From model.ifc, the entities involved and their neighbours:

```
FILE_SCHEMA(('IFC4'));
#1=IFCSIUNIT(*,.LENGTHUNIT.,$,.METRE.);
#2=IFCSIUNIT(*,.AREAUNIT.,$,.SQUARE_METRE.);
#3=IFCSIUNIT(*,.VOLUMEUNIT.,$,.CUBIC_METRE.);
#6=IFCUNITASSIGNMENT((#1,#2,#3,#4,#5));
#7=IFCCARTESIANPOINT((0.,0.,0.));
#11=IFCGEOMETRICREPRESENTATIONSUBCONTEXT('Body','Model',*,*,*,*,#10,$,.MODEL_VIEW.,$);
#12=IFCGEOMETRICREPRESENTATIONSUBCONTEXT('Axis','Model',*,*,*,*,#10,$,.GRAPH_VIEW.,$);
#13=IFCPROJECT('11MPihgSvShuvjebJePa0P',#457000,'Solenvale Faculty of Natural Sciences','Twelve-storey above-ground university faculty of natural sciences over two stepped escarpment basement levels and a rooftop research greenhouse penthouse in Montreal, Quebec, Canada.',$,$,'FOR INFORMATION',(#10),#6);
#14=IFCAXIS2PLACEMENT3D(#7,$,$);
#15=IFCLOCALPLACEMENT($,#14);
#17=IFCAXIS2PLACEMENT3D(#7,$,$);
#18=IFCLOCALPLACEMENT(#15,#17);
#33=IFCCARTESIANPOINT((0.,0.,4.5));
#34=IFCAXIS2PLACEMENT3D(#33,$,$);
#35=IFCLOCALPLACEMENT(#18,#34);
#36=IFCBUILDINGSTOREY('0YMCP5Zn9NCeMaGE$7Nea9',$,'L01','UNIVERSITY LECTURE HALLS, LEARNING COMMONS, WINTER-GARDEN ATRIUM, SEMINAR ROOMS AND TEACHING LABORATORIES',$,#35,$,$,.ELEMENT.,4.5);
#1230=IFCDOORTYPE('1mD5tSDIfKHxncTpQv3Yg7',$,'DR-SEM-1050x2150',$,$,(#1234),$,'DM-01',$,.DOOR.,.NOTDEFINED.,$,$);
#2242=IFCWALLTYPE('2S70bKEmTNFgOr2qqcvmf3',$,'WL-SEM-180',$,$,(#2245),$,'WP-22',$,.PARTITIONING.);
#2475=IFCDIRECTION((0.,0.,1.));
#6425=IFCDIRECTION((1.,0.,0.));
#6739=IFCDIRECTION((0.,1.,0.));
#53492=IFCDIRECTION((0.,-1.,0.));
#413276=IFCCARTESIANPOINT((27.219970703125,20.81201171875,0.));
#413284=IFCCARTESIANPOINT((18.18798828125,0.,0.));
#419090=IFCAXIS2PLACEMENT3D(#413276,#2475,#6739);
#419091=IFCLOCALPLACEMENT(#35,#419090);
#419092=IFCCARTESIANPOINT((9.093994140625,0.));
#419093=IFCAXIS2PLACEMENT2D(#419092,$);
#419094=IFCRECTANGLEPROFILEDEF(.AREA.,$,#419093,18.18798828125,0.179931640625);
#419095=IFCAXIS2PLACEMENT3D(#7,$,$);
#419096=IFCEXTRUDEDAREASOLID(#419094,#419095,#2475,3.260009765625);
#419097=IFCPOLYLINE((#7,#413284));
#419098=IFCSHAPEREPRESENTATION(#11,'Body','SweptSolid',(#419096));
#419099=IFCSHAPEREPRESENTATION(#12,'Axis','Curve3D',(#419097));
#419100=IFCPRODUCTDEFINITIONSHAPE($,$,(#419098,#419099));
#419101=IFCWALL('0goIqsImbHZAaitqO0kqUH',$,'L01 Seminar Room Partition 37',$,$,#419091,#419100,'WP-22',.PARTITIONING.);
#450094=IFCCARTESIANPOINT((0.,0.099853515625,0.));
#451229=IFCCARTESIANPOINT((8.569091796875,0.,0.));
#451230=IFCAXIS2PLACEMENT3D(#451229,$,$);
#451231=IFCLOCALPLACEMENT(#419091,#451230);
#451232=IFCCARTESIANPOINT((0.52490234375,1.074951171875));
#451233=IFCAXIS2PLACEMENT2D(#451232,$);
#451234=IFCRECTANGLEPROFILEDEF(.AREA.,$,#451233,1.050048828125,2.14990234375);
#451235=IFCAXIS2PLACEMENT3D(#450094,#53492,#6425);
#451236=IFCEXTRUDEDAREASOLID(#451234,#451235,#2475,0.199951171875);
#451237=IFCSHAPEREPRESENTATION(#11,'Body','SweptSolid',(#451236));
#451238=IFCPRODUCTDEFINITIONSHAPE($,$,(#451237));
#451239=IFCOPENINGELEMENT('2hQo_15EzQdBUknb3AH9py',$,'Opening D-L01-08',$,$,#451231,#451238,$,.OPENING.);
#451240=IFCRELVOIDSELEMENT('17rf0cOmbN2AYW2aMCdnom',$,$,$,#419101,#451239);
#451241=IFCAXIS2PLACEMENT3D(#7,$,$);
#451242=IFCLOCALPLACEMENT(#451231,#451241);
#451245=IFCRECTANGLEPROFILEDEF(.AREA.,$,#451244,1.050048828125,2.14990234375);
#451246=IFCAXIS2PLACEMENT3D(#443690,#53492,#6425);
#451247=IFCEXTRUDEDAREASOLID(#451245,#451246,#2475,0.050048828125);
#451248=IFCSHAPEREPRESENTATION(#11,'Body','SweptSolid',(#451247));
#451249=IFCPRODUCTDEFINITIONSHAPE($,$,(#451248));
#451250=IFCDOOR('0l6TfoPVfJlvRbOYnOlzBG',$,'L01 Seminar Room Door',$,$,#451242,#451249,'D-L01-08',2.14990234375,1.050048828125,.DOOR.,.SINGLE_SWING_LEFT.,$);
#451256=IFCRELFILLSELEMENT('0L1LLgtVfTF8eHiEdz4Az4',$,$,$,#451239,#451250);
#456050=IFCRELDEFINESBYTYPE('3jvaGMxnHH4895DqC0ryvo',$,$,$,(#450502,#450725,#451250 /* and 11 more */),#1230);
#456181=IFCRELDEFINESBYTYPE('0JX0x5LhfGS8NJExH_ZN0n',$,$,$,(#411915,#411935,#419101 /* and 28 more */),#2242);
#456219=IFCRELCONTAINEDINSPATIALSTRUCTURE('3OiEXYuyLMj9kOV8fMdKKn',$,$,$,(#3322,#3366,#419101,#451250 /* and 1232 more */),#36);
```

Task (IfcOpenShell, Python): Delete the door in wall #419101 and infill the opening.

```python
import ifcopenshell
import ifcopenshell.api.feature
import ifcopenshell.api.root
import ifcopenshell.geom
import ifcopenshell.util.shape

model = ifcopenshell.open("model.ifc")
settings = ifcopenshell.geom.settings()


def volume(element):
    """Net volume in cubic metres, openings subtracted."""
    shape = ifcopenshell.geom.create_shape(settings, element)
    return ifcopenshell.util.shape.get_volume(shape.geometry)


door = model.by_guid("0l6TfoPVfJlvRbOYnOlzBG")
opening = door.FillsVoids[0].RelatingOpeningElement
wall = opening.VoidsElements[0].RelatingBuildingElement
before = volume(wall)

ifcopenshell.api.root.remove_product(model, product=door)
ifcopenshell.api.feature.remove_feature(model, feature=opening)

after = volume(wall)

print(f"wall volume {before:.3f} -> {after:.3f} m3")

model.write("model_v2.ifc")
```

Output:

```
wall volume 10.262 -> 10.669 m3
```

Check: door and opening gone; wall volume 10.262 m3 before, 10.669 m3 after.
